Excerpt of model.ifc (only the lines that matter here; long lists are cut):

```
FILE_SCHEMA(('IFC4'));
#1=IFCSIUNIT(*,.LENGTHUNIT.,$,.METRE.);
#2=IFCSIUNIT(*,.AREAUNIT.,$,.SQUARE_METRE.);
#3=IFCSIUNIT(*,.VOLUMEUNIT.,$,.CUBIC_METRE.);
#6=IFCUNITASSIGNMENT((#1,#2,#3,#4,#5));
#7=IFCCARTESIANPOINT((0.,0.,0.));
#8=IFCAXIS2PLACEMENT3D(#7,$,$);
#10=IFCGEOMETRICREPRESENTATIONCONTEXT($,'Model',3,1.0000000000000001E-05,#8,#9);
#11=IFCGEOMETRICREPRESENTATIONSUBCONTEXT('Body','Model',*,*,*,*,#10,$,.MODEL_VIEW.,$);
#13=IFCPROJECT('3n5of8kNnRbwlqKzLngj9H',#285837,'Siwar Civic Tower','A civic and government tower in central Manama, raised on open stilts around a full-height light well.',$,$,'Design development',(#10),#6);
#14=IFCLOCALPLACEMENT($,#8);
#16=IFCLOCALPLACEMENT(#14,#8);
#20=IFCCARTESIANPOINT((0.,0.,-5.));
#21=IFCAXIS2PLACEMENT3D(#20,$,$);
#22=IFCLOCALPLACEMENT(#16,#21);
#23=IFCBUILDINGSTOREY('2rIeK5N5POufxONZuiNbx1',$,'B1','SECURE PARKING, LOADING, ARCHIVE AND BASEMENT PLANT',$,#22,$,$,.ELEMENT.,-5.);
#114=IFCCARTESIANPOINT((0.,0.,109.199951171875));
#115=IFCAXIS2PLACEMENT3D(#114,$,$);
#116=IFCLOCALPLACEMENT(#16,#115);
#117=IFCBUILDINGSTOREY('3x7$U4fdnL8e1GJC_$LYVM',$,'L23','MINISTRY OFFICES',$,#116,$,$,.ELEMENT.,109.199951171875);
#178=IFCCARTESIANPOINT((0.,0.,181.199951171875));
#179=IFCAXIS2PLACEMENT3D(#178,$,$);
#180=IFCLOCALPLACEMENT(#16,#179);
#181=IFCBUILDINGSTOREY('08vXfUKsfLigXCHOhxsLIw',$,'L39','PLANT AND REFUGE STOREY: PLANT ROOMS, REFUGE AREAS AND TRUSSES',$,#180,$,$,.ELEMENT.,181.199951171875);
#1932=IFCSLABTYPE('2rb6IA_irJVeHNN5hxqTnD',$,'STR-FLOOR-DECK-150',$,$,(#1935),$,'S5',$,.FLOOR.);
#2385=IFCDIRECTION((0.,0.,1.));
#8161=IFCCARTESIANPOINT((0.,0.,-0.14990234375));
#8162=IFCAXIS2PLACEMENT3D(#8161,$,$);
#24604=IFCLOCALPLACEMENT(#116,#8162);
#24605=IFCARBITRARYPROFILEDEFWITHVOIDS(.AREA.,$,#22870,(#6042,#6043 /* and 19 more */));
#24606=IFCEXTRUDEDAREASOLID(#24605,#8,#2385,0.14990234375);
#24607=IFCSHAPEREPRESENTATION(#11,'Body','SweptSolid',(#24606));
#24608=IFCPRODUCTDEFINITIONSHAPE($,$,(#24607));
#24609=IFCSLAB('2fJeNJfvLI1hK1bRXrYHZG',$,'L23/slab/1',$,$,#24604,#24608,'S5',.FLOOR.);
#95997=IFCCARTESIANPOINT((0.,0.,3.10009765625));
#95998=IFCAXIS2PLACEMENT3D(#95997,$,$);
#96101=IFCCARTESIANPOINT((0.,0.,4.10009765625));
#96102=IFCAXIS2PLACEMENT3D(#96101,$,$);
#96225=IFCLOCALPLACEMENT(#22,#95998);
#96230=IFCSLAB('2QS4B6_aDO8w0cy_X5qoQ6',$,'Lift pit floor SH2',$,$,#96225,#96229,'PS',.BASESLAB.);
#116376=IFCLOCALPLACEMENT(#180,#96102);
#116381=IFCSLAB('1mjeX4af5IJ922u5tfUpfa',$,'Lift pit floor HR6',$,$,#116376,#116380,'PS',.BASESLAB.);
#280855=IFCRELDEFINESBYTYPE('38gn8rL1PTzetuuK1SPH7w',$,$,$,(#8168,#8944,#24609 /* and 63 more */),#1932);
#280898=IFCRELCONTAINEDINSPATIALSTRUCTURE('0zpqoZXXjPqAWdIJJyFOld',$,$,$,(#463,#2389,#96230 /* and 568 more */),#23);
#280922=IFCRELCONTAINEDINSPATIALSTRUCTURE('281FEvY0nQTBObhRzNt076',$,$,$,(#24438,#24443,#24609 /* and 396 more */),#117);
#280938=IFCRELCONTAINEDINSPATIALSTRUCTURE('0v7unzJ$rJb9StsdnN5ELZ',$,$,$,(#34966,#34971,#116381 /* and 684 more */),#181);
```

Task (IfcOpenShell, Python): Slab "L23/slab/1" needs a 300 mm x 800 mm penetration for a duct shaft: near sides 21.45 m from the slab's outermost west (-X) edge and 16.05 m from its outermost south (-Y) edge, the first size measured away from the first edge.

```python
import numpy as np
import ifcopenshell
import ifcopenshell.api.feature
import ifcopenshell.api.geometry
import ifcopenshell.api.root
import ifcopenshell.geom
import ifcopenshell.util.placement
import ifcopenshell.util.representation
import ifcopenshell.util.shape
import ifcopenshell.util.unit

model = ifcopenshell.open("model.ifc")
unit_scale = ifcopenshell.util.unit.calculate_unit_scale(model)
settings = ifcopenshell.geom.settings()


def volume(element):
    """Net volume in cubic metres, openings subtracted."""
    shape = ifcopenshell.geom.create_shape(settings, element)
    return ifcopenshell.util.shape.get_volume(shape.geometry)


slab = model.by_id(24609)
before = volume(slab)

# Extent in the slab's own axes, in metres. The edges named are its -X and -Y sides.
slab_shape = ifcopenshell.geom.create_shape(settings, slab)
vertices = ifcopenshell.util.shape.get_vertices(slab_shape.geometry)
x_min, y_min, bottom = vertices.min(axis=0)
top = vertices[:, 2].max()

opening = ifcopenshell.api.root.create_entity(model, ifc_class="IfcOpeningElement", name="Duct shaft opening", predefined_type="OPENING")
context = ifcopenshell.util.representation.get_context(model, "Model", "Body", "MODEL_VIEW")
width, depth = 0.3, 0.8
outline = [(0.0, 0.0), (width, 0.0), (width, depth), (0.0, depth), (0.0, 0.0)]
# Overshoot both faces by 50 mm so the cut is clean.
shape = ifcopenshell.api.geometry.add_slab_representation(
    model, context=context, depth=top - bottom + 0.1, polyline=outline
)
ifcopenshell.api.geometry.assign_representation(model, product=opening, representation=shape)

matrix = ifcopenshell.util.placement.get_local_placement(slab.ObjectPlacement)
matrix[:, 3] = matrix @ np.append(np.array([x_min + 21.45, y_min + 16.05, bottom - 0.05]) / unit_scale, 1.0)
ifcopenshell.api.geometry.edit_object_placement(model, product=opening, matrix=matrix, is_si=False)
ifcopenshell.api.feature.add_feature(model, feature=opening, element=slab)

after = volume(slab)

print(f"slab volume {before:.3f} -> {after:.3f} m3")

model.write("model_v2.ifc")
```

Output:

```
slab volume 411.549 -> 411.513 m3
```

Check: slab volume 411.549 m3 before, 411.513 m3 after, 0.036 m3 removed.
